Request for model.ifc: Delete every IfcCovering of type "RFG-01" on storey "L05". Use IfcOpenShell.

First a look at what the model holds.

```python
import ifcopenshell
import ifcopenshell.util.element

model = ifcopenshell.open("model.ifc")
print(model.schema)
storey = next(s for s in model.by_type("IfcBuildingStorey") if s.Name == "L05")
coverings = [e for e in ifcopenshell.util.element.get_decomposition(storey) if e.is_a("IfcCovering")]
seen = {}
for e in coverings:
    element_type = ifcopenshell.util.element.get_type(e)
    name = element_type.Name if element_type not in (None, e) else None
    seen[name] = seen.get(name, 0) + 1
for name, count in sorted(seen.items(), key=str):
    print(count, "x", name)
```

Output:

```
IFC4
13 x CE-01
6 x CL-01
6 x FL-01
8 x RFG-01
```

```python
import ifcopenshell
import ifcopenshell.api.root
import ifcopenshell.util.element

model = ifcopenshell.open("model.ifc")

storey = next(s for s in model.by_type("IfcBuildingStorey") if s.Name == "L05")
coverings = [e for e in ifcopenshell.util.element.get_decomposition(storey) if e.is_a("IfcCovering")]
targets = [e for e in coverings if (t := ifcopenshell.util.element.get_type(e)) not in (None, e) and t.Name == "RFG-01"]

for e in targets:
    ifcopenshell.api.root.remove_product(model, product=e)
print(len(targets), "removed")

model.write("model_rev.ifc")
```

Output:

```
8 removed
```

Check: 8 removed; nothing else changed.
